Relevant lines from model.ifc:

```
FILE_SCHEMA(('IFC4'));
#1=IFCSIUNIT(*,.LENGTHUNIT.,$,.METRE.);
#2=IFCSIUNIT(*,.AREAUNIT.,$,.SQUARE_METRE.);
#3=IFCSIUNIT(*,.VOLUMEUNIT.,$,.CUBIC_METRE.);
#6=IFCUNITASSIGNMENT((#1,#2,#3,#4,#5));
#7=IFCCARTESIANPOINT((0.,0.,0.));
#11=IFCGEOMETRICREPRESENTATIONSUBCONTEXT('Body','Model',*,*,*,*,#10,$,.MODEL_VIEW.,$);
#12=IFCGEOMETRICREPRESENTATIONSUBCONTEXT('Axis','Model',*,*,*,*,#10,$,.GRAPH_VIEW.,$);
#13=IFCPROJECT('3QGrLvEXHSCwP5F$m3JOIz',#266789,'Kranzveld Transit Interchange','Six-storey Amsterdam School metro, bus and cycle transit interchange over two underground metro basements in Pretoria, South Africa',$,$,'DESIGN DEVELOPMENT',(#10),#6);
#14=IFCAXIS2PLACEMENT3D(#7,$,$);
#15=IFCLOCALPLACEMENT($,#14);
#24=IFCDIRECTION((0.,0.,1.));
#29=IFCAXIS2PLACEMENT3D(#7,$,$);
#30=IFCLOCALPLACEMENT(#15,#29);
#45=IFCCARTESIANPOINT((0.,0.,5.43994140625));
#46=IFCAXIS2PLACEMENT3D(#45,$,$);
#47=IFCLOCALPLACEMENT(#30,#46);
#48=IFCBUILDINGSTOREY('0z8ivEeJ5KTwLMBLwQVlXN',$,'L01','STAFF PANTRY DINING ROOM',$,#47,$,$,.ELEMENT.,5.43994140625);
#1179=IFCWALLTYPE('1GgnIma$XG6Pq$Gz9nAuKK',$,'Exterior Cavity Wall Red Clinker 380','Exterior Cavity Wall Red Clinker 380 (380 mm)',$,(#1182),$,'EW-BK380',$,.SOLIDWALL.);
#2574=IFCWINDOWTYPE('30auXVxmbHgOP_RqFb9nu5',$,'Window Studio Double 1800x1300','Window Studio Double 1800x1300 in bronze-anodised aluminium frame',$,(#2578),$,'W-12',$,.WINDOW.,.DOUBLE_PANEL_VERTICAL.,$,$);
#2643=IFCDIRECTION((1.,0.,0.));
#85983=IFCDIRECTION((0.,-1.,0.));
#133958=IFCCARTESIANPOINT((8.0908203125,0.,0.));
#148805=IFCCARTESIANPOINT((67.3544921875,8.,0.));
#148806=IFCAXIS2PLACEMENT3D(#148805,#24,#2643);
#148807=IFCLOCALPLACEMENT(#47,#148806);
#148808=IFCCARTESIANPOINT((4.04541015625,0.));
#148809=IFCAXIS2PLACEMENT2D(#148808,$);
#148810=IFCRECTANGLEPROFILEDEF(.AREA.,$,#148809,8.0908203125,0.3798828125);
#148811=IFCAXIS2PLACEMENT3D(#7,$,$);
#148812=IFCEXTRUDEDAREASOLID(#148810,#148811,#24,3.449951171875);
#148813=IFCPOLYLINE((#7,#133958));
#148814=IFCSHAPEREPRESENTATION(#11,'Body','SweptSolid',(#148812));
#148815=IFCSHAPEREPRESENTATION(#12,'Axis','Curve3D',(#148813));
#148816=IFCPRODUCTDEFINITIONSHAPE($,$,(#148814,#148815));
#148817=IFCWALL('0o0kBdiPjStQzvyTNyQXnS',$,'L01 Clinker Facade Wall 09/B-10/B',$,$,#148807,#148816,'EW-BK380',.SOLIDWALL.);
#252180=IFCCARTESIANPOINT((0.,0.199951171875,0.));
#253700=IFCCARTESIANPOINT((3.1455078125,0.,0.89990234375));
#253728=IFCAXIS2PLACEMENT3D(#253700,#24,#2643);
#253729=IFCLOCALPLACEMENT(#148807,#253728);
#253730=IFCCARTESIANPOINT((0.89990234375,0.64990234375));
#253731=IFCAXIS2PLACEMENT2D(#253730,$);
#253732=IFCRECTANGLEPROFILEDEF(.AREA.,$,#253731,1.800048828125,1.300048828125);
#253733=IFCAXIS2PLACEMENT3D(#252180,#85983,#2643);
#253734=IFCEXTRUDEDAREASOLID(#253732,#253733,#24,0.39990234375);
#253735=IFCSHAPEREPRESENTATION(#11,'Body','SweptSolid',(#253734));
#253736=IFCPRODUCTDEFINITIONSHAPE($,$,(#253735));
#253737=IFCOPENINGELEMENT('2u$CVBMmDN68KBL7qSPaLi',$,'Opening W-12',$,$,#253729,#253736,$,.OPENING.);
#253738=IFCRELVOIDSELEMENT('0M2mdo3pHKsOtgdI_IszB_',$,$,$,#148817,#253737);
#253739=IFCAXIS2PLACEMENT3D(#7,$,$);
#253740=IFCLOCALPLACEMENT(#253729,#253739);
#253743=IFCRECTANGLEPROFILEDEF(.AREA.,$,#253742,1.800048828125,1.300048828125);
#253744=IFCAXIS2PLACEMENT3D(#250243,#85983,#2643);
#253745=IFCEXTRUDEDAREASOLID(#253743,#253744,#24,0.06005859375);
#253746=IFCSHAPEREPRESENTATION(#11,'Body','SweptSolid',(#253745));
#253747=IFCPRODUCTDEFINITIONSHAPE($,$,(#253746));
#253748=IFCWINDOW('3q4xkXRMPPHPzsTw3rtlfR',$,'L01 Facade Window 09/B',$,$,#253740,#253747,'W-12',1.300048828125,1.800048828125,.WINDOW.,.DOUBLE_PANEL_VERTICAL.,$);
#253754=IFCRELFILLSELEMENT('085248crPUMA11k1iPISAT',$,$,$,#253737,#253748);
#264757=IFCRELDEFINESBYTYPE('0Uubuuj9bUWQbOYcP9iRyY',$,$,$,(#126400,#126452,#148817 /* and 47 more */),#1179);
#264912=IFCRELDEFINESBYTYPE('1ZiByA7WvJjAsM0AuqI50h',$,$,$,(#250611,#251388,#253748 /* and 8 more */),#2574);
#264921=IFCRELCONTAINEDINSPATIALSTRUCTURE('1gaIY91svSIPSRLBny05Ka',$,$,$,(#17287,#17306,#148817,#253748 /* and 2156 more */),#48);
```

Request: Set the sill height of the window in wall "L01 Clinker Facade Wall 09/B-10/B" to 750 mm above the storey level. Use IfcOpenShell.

```python
import numpy as np
import ifcopenshell
import ifcopenshell.api.geometry
import ifcopenshell.geom
import ifcopenshell.util.element
import ifcopenshell.util.placement
import ifcopenshell.util.shape
import ifcopenshell.util.unit

model = ifcopenshell.open("model.ifc")
unit_scale = ifcopenshell.util.unit.calculate_unit_scale(model)

window = model.by_guid("3q4xkXRMPPHPzsTw3rtlfR")
opening = window.FillsVoids[0].RelatingOpeningElement
storey = ifcopenshell.util.element.get_container(window, ifc_class="IfcBuildingStorey")
level = ifcopenshell.util.placement.get_local_placement(storey.ObjectPlacement)[2, 3]

# The opening's origin need not be at the sill, so measure its lowest point.
shape = ifcopenshell.geom.create_shape(ifcopenshell.geom.settings(), opening)
bottom = ifcopenshell.util.shape.get_shape_bottom_elevation(shape, shape.geometry) / unit_scale
dz = level + 0.75 / unit_scale - bottom

shift = np.array([0.0, 0.0, dz])
# The window is placed relative to its opening, so it follows when the opening moves.
matrix = ifcopenshell.util.placement.get_local_placement(opening.ObjectPlacement)
matrix[:3, 3] += shift
ifcopenshell.api.geometry.edit_object_placement(
    model, product=opening, matrix=matrix, is_si=False, should_transform_children=True
)

print(f"moved by {dz * unit_scale:+.3f} m")

model.write("model_rev.ifc")
```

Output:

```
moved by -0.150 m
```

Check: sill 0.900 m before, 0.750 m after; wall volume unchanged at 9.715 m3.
